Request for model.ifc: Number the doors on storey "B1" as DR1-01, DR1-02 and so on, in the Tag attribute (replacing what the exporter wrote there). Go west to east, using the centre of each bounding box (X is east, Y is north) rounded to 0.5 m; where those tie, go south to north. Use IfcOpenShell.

First a look at what the model holds.

```python
import ifcopenshell
import ifcopenshell.util.element
import ifcopenshell.util.placement

model = ifcopenshell.open("model.ifc")
print(model.schema)
storey = next(s for s in model.by_type("IfcBuildingStorey") if s.Name == "B1")
doors = [e for e in ifcopenshell.util.element.get_decomposition(storey) if e.is_a("IfcDoor")]
for e in sorted(doors, key=lambda e: e.id()):
    origin = ifcopenshell.util.placement.get_local_placement(e.ObjectPlacement)[:3, 3]
    print(e.id(), e.Tag, e.Name, origin.round(2) + 0.0, sep=" | ")
```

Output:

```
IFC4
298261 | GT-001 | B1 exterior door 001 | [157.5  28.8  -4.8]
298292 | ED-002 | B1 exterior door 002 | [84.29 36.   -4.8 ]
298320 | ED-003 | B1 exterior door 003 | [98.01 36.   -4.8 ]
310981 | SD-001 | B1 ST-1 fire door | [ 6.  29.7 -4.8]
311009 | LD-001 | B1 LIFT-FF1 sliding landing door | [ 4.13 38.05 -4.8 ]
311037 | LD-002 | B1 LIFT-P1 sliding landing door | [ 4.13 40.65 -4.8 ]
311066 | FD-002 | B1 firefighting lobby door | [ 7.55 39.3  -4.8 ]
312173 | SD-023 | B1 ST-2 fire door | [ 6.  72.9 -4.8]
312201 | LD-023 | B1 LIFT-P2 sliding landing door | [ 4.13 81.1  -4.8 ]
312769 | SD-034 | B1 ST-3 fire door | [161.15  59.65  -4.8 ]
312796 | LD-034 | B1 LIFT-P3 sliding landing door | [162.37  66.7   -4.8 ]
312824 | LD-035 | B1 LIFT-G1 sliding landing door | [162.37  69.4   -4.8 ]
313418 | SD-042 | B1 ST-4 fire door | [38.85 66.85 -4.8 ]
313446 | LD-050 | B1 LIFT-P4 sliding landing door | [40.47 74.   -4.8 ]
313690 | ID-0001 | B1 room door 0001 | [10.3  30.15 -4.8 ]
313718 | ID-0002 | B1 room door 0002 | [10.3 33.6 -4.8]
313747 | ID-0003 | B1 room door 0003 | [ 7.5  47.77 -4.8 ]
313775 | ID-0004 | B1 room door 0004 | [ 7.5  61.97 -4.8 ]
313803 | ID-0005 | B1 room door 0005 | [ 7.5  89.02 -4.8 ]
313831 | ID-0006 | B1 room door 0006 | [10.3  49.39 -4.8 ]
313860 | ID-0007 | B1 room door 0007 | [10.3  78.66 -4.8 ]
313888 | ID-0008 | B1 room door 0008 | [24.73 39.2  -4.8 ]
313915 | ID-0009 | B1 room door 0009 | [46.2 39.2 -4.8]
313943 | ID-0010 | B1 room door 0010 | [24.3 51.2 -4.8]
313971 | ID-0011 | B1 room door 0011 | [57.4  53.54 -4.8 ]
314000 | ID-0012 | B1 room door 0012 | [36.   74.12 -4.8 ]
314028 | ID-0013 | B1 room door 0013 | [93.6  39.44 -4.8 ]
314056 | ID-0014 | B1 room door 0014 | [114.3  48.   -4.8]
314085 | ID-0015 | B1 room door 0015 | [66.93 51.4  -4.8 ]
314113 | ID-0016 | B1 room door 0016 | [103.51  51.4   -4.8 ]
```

```python
import ifcopenshell
import ifcopenshell.geom
import ifcopenshell.util.element
import ifcopenshell.util.shape

model = ifcopenshell.open("model.ifc")
settings = ifcopenshell.geom.settings()
settings.set("use-world-coords", True)


def centre(element):
    shape = ifcopenshell.geom.create_shape(settings, element)
    return ifcopenshell.util.shape.get_bbox_centroid(shape.geometry)


storey = next(s for s in model.by_type("IfcBuildingStorey") if s.Name == "B1")
doors = [e for e in ifcopenshell.util.element.get_decomposition(storey) if e.is_a("IfcDoor")]

# Insertion points can sit at a corner or the storey origin, so sort by the geometry (in metres).
centres = {e: centre(e) for e in doors}
doors.sort(key=lambda e: (round(centres[e][0] / 0.5), centres[e][1]))

for i, e in enumerate(doors, start=1):
    number = f"DR1-{i:02d}"
    e.Tag = number
    print(e.id(), number)

model.write("model_v2.ifc")
```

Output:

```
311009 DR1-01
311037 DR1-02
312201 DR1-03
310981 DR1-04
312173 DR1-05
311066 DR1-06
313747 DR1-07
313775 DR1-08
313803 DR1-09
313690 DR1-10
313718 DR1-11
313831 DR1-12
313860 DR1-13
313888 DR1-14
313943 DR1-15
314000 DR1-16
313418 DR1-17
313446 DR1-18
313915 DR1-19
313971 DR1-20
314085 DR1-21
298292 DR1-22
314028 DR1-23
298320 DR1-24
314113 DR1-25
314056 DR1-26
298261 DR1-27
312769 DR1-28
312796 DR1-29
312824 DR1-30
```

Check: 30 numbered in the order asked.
